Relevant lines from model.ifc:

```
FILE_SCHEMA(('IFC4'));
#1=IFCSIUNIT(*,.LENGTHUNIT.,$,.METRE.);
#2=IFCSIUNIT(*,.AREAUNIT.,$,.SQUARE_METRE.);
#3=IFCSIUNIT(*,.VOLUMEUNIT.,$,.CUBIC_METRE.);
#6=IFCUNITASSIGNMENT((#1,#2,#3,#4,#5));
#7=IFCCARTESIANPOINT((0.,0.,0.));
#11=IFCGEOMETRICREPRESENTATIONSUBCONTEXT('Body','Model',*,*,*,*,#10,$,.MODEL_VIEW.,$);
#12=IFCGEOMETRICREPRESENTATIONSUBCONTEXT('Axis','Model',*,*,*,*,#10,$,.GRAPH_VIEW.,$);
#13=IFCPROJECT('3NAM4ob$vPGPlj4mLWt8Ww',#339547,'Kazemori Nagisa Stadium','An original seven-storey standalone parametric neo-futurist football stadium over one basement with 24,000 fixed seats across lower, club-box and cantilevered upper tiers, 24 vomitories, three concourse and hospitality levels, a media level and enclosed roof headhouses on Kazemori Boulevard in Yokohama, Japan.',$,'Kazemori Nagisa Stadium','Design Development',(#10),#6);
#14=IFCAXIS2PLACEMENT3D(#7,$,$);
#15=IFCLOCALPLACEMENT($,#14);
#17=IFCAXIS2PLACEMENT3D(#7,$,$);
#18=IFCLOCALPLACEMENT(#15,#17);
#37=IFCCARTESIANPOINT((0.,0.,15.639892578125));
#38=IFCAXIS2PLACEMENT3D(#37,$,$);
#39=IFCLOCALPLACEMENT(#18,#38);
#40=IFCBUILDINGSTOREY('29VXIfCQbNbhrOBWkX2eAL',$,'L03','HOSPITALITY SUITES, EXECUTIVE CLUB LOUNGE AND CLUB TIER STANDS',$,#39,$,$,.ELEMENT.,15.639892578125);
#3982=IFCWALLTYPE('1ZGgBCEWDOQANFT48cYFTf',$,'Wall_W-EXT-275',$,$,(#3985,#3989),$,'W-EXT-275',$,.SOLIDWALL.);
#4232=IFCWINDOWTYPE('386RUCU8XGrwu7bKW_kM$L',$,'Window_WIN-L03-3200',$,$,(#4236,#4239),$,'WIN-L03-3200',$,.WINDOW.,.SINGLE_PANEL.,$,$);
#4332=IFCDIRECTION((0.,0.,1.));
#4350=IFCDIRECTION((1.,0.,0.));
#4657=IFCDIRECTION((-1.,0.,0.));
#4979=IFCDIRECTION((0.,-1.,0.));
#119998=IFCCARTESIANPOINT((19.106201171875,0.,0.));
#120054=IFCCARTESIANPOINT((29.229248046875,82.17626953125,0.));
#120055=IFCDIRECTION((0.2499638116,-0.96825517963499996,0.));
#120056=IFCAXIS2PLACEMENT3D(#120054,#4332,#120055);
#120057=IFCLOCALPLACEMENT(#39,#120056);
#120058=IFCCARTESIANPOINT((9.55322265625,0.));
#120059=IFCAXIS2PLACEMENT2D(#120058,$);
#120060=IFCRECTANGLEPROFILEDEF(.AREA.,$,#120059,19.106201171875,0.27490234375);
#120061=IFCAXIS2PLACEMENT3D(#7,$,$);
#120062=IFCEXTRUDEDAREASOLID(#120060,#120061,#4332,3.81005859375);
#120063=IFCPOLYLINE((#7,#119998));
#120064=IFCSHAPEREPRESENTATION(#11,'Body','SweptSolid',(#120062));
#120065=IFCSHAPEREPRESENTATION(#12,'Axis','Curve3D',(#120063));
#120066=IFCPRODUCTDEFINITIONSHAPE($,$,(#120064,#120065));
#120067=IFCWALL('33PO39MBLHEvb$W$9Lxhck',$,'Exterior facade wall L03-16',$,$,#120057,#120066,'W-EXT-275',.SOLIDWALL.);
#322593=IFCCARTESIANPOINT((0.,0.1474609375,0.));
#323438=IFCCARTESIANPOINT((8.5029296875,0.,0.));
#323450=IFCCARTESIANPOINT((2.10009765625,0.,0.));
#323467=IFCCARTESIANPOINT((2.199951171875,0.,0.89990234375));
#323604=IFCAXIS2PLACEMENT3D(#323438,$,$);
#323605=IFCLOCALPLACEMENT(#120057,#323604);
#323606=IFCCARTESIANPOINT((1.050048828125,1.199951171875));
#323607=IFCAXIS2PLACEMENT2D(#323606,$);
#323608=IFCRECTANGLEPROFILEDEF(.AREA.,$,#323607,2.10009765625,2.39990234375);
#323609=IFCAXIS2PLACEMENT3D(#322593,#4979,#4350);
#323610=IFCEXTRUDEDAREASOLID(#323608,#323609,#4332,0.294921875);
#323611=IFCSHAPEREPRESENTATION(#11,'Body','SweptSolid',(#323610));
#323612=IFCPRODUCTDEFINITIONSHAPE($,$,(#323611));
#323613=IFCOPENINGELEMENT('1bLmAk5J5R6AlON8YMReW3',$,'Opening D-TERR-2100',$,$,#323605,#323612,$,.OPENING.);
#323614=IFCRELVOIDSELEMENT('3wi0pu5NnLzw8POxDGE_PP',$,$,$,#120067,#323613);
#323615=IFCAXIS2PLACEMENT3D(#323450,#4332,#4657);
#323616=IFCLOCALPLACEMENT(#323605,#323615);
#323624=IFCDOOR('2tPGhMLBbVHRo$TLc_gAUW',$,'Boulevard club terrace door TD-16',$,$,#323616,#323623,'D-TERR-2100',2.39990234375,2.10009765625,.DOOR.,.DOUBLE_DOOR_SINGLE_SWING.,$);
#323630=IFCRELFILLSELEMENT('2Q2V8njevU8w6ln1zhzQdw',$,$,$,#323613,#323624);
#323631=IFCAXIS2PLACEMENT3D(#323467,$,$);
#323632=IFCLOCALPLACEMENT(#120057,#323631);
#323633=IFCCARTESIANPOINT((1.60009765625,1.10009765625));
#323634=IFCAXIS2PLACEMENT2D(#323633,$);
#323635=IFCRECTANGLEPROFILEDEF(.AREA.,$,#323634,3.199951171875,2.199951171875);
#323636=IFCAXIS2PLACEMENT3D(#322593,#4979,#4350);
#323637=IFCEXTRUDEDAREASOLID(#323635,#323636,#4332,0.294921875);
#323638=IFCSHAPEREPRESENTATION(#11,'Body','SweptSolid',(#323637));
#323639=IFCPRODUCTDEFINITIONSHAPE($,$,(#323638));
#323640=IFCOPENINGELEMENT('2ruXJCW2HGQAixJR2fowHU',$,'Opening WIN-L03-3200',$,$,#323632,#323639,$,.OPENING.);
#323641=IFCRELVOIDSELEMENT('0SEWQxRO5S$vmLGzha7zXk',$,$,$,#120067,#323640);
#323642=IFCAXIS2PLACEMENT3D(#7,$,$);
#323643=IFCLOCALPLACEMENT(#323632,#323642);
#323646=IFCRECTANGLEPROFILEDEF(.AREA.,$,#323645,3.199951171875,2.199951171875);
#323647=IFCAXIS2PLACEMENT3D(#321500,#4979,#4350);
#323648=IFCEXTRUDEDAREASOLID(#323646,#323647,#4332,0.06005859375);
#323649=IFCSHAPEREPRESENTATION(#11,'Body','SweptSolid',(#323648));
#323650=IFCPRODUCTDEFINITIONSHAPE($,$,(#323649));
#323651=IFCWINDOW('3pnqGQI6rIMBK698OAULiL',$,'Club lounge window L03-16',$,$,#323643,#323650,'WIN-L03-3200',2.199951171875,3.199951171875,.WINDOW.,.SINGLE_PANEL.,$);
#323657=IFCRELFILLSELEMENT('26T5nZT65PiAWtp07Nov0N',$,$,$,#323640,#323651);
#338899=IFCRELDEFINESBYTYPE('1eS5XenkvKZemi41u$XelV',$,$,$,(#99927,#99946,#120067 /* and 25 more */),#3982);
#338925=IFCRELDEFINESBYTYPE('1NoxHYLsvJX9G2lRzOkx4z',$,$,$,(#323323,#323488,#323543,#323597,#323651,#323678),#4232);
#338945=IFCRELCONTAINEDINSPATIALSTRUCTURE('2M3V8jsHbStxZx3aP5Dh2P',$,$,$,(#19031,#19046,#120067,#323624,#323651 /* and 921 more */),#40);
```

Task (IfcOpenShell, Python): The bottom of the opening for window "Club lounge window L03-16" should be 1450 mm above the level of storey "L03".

```python
import numpy as np
import ifcopenshell
import ifcopenshell.api.geometry
import ifcopenshell.geom
import ifcopenshell.util.element
import ifcopenshell.util.placement
import ifcopenshell.util.shape
import ifcopenshell.util.unit

model = ifcopenshell.open("model.ifc")
unit_scale = ifcopenshell.util.unit.calculate_unit_scale(model)

window = model.by_guid("3pnqGQI6rIMBK698OAULiL")
opening = window.FillsVoids[0].RelatingOpeningElement
storey = ifcopenshell.util.element.get_container(window, ifc_class="IfcBuildingStorey")
level = ifcopenshell.util.placement.get_local_placement(storey.ObjectPlacement)[2, 3]

# The opening's origin need not be at the sill, so measure its lowest point.
shape = ifcopenshell.geom.create_shape(ifcopenshell.geom.settings(), opening)
bottom = ifcopenshell.util.shape.get_shape_bottom_elevation(shape, shape.geometry) / unit_scale
dz = level + 1.45 / unit_scale - bottom

shift = np.array([0.0, 0.0, dz])
# The window is placed relative to its opening, so it follows when the opening moves.
matrix = ifcopenshell.util.placement.get_local_placement(opening.ObjectPlacement)
matrix[:3, 3] += shift
ifcopenshell.api.geometry.edit_object_placement(
    model, product=opening, matrix=matrix, is_si=False, should_transform_children=True
)

print(f"moved by {dz * unit_scale:+.3f} m")

model.write("model-out.ifc")
```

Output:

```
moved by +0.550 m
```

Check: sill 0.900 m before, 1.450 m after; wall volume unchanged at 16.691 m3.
